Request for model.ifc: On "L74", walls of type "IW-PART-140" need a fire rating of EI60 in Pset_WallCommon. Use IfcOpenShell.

First a look at what the model holds.

```python
import ifcopenshell
import ifcopenshell.util.element

model = ifcopenshell.open("model.ifc")
print(model.schema)
storey = next(s for s in model.by_type("IfcBuildingStorey") if s.Name == "L74")
walls = [e for e in ifcopenshell.util.element.get_decomposition(storey) if e.is_a("IfcWall")]
seen = {}
for e in walls:
    element_type = ifcopenshell.util.element.get_type(e)
    key = (element_type.Name if element_type != e and element_type else None, ifcopenshell.util.element.get_pset(e, "Pset_WallCommon", "FireRating"))
    seen[key] = seen.get(key, 0) + 1
for (name, value), count in sorted(seen.items(), key=str):
    print(count, "x", name, "|", value)
```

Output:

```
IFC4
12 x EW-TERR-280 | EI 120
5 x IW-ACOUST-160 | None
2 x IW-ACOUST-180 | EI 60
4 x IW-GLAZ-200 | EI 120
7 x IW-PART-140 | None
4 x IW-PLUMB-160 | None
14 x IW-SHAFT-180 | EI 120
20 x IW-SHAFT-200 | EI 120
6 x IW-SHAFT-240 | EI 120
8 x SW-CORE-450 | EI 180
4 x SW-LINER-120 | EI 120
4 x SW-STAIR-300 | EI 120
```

```python
import ifcopenshell
import ifcopenshell.api.pset
import ifcopenshell.util.element

model = ifcopenshell.open("model.ifc")

storey = next(s for s in model.by_type("IfcBuildingStorey") if s.Name == "L74")
walls = [e for e in ifcopenshell.util.element.get_decomposition(storey) if e.is_a("IfcWall")]

count = 0
for e in walls:
    element_type = ifcopenshell.util.element.get_type(e)
    if element_type in (None, e) or element_type.Name != "IW-PART-140":
        continue
    found = ifcopenshell.util.element.get_pset(e, "Pset_WallCommon", should_inherit=False)
    if found:
        pset = model.by_id(found["id"])
        if len(ifcopenshell.util.element.get_elements_by_pset(pset)) > 1:
            pset = ifcopenshell.api.pset.unshare_pset(model, products=[e], pset=pset)[0]
    else:
        pset = ifcopenshell.api.pset.add_pset(model, product=e, name="Pset_WallCommon")
    ifcopenshell.api.pset.edit_pset(model, pset=pset, properties={"FireRating": "EI60"})
    count += 1

print(count, "walls updated")

model.write("model_rev.ifc")
```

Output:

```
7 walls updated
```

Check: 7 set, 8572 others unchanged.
